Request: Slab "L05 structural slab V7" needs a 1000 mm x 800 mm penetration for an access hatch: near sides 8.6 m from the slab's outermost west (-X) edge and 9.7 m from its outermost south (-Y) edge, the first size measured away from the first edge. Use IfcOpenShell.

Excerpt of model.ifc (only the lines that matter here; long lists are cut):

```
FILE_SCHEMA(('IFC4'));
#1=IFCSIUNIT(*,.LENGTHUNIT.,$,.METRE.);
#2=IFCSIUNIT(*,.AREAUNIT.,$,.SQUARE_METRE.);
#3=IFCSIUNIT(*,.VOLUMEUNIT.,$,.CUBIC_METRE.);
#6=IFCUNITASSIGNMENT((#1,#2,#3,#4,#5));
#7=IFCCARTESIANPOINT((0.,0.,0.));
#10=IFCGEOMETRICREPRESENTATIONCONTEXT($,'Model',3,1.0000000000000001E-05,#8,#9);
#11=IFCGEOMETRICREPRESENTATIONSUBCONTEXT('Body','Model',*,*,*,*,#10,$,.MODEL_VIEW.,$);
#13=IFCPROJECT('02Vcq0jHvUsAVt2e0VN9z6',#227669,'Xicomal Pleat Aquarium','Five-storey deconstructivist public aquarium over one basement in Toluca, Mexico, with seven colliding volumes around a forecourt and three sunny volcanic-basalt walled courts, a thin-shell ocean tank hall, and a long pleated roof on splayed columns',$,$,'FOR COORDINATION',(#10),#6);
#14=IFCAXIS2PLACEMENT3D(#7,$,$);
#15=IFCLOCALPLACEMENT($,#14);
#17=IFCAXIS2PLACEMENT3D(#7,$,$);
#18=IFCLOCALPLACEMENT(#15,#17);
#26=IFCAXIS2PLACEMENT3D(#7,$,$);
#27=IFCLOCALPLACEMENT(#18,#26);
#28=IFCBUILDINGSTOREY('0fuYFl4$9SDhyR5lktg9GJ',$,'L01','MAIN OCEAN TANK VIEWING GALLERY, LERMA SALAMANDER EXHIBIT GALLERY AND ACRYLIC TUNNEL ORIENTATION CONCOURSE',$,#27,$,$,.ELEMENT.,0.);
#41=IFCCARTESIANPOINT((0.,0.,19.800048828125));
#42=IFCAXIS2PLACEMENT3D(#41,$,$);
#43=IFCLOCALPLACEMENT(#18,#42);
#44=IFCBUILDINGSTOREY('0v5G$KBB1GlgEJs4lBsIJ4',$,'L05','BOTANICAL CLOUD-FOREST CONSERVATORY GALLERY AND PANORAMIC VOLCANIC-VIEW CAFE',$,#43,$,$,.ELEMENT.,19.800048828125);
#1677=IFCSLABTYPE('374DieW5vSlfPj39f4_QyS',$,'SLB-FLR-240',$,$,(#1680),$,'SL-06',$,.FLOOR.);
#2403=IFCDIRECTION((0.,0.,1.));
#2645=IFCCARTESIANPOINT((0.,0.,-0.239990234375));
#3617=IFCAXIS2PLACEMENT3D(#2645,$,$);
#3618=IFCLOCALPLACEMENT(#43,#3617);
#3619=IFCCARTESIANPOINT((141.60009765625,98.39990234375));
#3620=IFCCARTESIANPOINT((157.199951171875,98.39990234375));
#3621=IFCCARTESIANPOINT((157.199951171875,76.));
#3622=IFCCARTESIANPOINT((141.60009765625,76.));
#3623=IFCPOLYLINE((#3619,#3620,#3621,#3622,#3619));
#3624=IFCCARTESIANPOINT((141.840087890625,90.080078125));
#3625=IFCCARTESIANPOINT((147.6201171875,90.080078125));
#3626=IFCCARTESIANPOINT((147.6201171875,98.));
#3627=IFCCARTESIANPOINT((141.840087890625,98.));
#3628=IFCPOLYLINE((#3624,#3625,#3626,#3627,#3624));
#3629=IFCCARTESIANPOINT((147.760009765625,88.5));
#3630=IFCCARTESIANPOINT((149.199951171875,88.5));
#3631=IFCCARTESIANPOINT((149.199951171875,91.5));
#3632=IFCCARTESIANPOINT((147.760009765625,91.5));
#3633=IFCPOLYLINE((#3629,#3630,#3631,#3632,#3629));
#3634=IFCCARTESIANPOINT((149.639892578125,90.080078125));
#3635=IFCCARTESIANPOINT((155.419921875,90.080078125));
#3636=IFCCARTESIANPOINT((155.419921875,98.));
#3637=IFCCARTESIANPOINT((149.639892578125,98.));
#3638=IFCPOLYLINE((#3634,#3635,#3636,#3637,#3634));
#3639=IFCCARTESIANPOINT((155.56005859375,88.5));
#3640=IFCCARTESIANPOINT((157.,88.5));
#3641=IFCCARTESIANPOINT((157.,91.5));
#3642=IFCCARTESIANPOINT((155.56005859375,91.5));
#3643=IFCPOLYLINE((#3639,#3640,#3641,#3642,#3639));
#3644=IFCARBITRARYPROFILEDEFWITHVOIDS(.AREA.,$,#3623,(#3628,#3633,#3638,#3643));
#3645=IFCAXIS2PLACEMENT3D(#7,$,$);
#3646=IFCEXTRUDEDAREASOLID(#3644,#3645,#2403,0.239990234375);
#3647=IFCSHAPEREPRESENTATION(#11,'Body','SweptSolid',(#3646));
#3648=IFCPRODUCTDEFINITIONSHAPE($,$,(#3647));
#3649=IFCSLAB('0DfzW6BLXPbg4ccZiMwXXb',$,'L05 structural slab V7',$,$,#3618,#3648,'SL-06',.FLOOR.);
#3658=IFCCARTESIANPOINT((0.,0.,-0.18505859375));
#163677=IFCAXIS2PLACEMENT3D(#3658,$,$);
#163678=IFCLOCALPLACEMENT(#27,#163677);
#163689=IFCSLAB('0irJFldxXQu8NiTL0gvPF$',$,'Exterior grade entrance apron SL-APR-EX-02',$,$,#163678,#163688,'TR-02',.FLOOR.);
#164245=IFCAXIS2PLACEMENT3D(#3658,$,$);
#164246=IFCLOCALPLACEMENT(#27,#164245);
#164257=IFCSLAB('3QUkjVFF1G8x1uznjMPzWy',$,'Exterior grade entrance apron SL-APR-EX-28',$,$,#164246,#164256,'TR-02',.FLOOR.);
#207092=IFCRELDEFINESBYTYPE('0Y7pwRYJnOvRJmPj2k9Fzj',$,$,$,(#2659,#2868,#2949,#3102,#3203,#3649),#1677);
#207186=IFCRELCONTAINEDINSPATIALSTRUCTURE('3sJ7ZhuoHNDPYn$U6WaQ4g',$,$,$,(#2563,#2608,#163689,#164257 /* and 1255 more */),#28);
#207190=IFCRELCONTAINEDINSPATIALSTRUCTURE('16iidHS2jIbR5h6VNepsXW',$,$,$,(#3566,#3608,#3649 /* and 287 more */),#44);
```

```python
import numpy as np
import ifcopenshell
import ifcopenshell.api.feature
import ifcopenshell.api.geometry
import ifcopenshell.api.root
import ifcopenshell.geom
import ifcopenshell.util.placement
import ifcopenshell.util.representation
import ifcopenshell.util.shape
import ifcopenshell.util.unit

model = ifcopenshell.open("model.ifc")
unit_scale = ifcopenshell.util.unit.calculate_unit_scale(model)
settings = ifcopenshell.geom.settings()


def volume(element):
    """Net volume in cubic metres, openings subtracted."""
    shape = ifcopenshell.geom.create_shape(settings, element)
    return ifcopenshell.util.shape.get_volume(shape.geometry)


slab = model.by_guid("0DfzW6BLXPbg4ccZiMwXXb")
before = volume(slab)

# Extent in the slab's own axes, in metres. The edges named are its -X and -Y sides.
slab_shape = ifcopenshell.geom.create_shape(settings, slab)
vertices = ifcopenshell.util.shape.get_vertices(slab_shape.geometry)
x_min, y_min, bottom = vertices.min(axis=0)
top = vertices[:, 2].max()

opening = ifcopenshell.api.root.create_entity(model, ifc_class="IfcOpeningElement", name="Access hatch opening", predefined_type="OPENING")
context = ifcopenshell.util.representation.get_context(model, "Model", "Body", "MODEL_VIEW")
width, depth = 1, 0.8
outline = [(0.0, 0.0), (width, 0.0), (width, depth), (0.0, depth), (0.0, 0.0)]
# Overshoot both faces by 50 mm so the cut is clean.
shape = ifcopenshell.api.geometry.add_slab_representation(
    model, context=context, depth=top - bottom + 0.1, polyline=outline
)
ifcopenshell.api.geometry.assign_representation(model, product=opening, representation=shape)

matrix = ifcopenshell.util.placement.get_local_placement(slab.ObjectPlacement)
matrix[:, 3] = matrix @ np.append(np.array([x_min + 8.6, y_min + 9.7, bottom - 0.05]) / unit_scale, 1.0)
ifcopenshell.api.geometry.edit_object_placement(model, product=opening, matrix=matrix, is_si=False)
ifcopenshell.api.feature.add_feature(model, feature=opening, element=slab)

after = volume(slab)

print(f"slab volume {before:.3f} -> {after:.3f} m3")

model.write("model-out.ifc")
```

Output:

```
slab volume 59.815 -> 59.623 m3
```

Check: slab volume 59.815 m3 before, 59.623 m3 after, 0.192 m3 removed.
